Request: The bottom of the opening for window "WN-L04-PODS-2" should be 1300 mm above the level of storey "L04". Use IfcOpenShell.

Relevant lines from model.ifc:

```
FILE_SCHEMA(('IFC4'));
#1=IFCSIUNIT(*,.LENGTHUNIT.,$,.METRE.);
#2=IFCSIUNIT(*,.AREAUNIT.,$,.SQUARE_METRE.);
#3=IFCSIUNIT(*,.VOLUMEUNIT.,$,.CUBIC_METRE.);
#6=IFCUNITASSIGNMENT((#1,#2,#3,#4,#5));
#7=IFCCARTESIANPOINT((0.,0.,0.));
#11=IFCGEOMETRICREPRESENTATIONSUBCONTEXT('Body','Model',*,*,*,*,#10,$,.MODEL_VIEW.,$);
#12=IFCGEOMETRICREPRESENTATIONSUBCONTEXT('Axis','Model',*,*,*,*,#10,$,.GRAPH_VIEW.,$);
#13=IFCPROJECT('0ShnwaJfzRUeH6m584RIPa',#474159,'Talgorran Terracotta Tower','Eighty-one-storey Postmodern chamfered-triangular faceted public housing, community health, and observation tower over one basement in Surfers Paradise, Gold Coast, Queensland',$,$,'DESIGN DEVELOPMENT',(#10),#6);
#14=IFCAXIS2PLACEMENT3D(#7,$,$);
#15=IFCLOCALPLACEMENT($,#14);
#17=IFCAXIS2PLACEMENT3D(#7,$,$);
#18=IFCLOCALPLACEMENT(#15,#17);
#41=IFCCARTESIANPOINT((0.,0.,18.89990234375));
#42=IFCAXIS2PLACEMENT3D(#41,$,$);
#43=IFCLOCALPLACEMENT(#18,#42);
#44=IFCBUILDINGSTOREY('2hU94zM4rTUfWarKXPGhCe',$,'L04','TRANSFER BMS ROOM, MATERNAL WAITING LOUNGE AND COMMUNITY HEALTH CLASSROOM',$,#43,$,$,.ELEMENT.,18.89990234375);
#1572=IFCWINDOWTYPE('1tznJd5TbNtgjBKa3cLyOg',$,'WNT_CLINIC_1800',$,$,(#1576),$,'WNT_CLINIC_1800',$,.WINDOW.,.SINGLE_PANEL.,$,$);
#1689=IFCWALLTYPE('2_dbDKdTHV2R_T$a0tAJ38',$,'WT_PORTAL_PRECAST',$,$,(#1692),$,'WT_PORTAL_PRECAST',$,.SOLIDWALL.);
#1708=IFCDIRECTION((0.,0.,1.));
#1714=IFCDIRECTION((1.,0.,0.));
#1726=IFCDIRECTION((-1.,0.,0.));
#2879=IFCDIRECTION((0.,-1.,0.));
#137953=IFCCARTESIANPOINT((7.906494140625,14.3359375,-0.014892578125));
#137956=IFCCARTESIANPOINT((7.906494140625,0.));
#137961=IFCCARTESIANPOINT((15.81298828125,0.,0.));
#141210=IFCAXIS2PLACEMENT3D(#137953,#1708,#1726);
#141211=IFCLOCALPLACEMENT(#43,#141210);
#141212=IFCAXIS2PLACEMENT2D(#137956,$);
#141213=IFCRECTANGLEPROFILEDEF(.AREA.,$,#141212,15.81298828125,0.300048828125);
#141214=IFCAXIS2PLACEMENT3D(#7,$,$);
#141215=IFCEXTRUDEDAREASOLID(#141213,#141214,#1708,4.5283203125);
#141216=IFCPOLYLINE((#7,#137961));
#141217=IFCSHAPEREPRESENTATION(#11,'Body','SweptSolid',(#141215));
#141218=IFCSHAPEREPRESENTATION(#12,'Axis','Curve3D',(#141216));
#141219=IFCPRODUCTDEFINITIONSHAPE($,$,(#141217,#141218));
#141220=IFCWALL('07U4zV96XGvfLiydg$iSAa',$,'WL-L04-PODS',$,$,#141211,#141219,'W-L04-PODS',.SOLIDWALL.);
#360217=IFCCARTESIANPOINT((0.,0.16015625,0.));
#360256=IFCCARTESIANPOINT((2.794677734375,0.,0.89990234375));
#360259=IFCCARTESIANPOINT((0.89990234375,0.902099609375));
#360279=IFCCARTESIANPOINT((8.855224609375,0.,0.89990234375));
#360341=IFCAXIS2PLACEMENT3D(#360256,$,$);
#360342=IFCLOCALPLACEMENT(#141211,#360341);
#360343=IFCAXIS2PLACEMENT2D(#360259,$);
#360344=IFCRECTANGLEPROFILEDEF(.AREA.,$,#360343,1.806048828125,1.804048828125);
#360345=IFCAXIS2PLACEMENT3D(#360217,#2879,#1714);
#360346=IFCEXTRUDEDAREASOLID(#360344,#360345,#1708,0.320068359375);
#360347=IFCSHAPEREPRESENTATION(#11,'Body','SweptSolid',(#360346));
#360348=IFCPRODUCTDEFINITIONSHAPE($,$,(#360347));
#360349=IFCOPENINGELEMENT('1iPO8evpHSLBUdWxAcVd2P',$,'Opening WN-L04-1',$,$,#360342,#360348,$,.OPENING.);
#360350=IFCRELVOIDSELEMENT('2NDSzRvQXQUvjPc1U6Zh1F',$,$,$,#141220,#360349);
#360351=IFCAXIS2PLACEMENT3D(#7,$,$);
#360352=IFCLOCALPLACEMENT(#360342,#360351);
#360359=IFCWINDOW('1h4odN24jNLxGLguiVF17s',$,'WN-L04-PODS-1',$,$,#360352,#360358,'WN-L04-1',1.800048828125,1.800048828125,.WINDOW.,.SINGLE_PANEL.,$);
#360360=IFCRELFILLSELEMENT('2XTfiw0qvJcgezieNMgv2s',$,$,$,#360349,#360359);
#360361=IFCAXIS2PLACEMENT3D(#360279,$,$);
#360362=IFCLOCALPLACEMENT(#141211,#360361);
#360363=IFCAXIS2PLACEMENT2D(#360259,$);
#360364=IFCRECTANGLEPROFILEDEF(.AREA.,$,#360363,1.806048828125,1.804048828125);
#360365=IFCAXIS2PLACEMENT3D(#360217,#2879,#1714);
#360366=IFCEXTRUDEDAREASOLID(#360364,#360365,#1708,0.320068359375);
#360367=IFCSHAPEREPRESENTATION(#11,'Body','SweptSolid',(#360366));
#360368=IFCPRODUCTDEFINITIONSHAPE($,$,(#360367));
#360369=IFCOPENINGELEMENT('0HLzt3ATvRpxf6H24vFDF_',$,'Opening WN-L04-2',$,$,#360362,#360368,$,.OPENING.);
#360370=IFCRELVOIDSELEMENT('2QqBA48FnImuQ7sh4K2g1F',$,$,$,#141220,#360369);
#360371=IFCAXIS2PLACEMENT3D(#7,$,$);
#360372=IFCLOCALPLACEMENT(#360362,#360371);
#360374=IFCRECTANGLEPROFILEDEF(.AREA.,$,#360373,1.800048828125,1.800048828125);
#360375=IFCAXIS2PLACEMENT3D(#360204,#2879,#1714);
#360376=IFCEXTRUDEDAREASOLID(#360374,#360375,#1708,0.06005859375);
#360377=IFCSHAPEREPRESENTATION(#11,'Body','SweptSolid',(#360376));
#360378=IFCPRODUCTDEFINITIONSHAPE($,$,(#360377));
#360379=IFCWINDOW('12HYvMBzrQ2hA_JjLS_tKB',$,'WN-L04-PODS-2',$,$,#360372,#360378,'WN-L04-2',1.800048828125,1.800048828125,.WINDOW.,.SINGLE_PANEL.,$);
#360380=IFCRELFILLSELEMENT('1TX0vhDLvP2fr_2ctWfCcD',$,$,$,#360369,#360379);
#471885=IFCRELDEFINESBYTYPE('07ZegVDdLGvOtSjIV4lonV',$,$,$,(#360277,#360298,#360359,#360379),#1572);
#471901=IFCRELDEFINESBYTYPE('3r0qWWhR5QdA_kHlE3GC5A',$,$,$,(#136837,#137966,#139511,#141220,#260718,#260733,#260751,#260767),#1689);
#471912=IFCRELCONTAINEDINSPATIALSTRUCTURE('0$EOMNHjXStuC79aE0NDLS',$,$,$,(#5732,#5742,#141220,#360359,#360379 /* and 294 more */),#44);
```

```python
import numpy as np
import ifcopenshell
import ifcopenshell.api.geometry
import ifcopenshell.geom
import ifcopenshell.util.element
import ifcopenshell.util.placement
import ifcopenshell.util.shape
import ifcopenshell.util.unit

model = ifcopenshell.open("model.ifc")
unit_scale = ifcopenshell.util.unit.calculate_unit_scale(model)

window = model.by_id(360379)
opening = window.FillsVoids[0].RelatingOpeningElement
storey = ifcopenshell.util.element.get_container(window, ifc_class="IfcBuildingStorey")
level = ifcopenshell.util.placement.get_local_placement(storey.ObjectPlacement)[2, 3]

# The opening's origin need not be at the sill, so measure its lowest point.
shape = ifcopenshell.geom.create_shape(ifcopenshell.geom.settings(), opening)
bottom = ifcopenshell.util.shape.get_shape_bottom_elevation(shape, shape.geometry) / unit_scale
dz = level + 1.3 / unit_scale - bottom

shift = np.array([0.0, 0.0, dz])
# The window is placed relative to its opening, so it follows when the opening moves.
matrix = ifcopenshell.util.placement.get_local_placement(opening.ObjectPlacement)
matrix[:3, 3] += shift
ifcopenshell.api.geometry.edit_object_placement(
    model, product=opening, matrix=matrix, is_si=False, should_transform_children=True
)

print(f"moved by {dz * unit_scale:+.3f} m")

model.write("model_v2.ifc")
```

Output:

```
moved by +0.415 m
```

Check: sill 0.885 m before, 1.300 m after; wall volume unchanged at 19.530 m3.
